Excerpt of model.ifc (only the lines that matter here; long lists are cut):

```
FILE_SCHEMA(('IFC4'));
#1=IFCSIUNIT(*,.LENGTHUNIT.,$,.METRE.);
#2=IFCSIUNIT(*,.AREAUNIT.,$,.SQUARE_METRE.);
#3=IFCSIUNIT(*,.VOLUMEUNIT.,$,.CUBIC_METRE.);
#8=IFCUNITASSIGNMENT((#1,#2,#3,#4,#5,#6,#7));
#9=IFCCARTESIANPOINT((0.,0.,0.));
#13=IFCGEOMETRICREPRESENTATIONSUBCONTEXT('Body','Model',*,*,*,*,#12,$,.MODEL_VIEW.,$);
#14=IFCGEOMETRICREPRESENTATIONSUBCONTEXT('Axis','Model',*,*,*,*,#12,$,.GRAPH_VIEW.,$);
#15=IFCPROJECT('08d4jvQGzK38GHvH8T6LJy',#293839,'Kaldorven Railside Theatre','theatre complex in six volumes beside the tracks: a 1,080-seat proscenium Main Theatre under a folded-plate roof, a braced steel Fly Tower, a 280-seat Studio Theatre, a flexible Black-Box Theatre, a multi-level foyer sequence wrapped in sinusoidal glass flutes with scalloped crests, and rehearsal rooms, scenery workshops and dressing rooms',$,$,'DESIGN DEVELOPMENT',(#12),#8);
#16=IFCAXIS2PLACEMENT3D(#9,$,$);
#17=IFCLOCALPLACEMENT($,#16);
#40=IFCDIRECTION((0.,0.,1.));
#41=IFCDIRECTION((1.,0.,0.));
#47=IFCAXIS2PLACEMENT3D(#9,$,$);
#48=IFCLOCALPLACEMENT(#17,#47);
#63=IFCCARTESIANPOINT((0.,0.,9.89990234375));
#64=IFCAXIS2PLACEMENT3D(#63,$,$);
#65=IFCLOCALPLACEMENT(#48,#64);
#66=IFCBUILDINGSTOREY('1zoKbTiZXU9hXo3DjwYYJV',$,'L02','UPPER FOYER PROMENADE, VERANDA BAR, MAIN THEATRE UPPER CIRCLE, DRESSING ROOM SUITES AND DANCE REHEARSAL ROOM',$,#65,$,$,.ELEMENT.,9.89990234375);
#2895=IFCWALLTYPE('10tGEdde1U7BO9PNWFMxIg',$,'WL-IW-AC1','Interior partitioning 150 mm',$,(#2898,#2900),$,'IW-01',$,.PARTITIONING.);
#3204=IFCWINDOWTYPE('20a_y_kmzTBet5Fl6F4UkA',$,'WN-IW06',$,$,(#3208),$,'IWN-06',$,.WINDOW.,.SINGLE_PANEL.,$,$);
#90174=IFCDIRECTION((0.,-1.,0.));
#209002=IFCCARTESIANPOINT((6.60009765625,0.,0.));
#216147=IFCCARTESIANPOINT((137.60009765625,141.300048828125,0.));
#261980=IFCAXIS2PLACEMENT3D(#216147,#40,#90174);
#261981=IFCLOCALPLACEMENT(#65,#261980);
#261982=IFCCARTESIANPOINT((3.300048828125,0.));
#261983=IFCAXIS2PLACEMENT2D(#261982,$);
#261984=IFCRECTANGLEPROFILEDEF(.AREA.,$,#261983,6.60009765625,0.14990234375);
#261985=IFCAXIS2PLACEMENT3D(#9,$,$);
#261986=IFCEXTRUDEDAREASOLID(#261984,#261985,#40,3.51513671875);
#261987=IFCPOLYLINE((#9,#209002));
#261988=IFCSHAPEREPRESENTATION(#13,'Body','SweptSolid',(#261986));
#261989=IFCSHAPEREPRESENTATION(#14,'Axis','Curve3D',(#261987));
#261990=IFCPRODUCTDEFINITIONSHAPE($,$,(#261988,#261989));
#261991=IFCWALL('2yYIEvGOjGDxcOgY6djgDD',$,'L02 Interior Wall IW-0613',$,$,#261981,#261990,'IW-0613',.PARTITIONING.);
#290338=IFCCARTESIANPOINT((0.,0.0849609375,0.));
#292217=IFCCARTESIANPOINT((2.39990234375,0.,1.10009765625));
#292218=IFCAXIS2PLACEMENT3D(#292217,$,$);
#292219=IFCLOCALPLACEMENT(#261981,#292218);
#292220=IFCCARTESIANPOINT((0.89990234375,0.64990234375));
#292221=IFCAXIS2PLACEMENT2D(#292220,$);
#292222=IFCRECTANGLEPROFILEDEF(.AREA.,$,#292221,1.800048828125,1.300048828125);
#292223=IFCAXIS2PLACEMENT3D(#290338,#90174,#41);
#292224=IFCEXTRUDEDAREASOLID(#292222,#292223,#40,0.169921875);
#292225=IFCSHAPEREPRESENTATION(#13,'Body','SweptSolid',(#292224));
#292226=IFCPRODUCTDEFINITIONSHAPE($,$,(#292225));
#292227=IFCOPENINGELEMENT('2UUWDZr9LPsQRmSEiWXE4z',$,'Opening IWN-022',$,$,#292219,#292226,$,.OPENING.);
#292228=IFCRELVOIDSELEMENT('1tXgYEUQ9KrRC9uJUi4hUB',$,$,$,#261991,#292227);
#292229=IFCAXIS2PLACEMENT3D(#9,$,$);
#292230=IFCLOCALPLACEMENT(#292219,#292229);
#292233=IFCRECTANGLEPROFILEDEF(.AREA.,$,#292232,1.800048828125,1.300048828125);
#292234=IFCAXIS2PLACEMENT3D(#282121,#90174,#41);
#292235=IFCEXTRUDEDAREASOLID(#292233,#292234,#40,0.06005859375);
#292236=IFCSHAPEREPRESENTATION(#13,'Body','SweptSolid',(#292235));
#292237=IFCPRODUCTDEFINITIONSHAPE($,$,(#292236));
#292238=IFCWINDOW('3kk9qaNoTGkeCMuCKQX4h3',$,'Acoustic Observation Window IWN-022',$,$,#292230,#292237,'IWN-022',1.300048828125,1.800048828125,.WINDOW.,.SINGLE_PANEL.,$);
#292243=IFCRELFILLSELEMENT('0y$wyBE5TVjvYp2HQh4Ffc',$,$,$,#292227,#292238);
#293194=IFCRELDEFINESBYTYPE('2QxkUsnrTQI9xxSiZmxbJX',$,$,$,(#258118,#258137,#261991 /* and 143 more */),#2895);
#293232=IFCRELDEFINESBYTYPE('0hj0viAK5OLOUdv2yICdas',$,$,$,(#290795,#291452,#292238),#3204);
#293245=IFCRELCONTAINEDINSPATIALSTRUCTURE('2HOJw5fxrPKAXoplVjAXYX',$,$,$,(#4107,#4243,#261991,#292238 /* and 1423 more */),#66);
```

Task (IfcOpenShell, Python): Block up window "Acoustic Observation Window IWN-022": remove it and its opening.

```python
import ifcopenshell
import ifcopenshell.api.feature
import ifcopenshell.api.root
import ifcopenshell.geom
import ifcopenshell.util.shape

model = ifcopenshell.open("model.ifc")
settings = ifcopenshell.geom.settings()


def volume(element):
    """Net volume in cubic metres, openings subtracted."""
    shape = ifcopenshell.geom.create_shape(settings, element)
    return ifcopenshell.util.shape.get_volume(shape.geometry)


window = model.by_id(292238)
opening = window.FillsVoids[0].RelatingOpeningElement
wall = opening.VoidsElements[0].RelatingBuildingElement
before = volume(wall)

ifcopenshell.api.root.remove_product(model, product=window)
ifcopenshell.api.feature.remove_feature(model, feature=opening)

after = volume(wall)

print(f"wall volume {before:.3f} -> {after:.3f} m3")

model.write("model_v2.ifc")
```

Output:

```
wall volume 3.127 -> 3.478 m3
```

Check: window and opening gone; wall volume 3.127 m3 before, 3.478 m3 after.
